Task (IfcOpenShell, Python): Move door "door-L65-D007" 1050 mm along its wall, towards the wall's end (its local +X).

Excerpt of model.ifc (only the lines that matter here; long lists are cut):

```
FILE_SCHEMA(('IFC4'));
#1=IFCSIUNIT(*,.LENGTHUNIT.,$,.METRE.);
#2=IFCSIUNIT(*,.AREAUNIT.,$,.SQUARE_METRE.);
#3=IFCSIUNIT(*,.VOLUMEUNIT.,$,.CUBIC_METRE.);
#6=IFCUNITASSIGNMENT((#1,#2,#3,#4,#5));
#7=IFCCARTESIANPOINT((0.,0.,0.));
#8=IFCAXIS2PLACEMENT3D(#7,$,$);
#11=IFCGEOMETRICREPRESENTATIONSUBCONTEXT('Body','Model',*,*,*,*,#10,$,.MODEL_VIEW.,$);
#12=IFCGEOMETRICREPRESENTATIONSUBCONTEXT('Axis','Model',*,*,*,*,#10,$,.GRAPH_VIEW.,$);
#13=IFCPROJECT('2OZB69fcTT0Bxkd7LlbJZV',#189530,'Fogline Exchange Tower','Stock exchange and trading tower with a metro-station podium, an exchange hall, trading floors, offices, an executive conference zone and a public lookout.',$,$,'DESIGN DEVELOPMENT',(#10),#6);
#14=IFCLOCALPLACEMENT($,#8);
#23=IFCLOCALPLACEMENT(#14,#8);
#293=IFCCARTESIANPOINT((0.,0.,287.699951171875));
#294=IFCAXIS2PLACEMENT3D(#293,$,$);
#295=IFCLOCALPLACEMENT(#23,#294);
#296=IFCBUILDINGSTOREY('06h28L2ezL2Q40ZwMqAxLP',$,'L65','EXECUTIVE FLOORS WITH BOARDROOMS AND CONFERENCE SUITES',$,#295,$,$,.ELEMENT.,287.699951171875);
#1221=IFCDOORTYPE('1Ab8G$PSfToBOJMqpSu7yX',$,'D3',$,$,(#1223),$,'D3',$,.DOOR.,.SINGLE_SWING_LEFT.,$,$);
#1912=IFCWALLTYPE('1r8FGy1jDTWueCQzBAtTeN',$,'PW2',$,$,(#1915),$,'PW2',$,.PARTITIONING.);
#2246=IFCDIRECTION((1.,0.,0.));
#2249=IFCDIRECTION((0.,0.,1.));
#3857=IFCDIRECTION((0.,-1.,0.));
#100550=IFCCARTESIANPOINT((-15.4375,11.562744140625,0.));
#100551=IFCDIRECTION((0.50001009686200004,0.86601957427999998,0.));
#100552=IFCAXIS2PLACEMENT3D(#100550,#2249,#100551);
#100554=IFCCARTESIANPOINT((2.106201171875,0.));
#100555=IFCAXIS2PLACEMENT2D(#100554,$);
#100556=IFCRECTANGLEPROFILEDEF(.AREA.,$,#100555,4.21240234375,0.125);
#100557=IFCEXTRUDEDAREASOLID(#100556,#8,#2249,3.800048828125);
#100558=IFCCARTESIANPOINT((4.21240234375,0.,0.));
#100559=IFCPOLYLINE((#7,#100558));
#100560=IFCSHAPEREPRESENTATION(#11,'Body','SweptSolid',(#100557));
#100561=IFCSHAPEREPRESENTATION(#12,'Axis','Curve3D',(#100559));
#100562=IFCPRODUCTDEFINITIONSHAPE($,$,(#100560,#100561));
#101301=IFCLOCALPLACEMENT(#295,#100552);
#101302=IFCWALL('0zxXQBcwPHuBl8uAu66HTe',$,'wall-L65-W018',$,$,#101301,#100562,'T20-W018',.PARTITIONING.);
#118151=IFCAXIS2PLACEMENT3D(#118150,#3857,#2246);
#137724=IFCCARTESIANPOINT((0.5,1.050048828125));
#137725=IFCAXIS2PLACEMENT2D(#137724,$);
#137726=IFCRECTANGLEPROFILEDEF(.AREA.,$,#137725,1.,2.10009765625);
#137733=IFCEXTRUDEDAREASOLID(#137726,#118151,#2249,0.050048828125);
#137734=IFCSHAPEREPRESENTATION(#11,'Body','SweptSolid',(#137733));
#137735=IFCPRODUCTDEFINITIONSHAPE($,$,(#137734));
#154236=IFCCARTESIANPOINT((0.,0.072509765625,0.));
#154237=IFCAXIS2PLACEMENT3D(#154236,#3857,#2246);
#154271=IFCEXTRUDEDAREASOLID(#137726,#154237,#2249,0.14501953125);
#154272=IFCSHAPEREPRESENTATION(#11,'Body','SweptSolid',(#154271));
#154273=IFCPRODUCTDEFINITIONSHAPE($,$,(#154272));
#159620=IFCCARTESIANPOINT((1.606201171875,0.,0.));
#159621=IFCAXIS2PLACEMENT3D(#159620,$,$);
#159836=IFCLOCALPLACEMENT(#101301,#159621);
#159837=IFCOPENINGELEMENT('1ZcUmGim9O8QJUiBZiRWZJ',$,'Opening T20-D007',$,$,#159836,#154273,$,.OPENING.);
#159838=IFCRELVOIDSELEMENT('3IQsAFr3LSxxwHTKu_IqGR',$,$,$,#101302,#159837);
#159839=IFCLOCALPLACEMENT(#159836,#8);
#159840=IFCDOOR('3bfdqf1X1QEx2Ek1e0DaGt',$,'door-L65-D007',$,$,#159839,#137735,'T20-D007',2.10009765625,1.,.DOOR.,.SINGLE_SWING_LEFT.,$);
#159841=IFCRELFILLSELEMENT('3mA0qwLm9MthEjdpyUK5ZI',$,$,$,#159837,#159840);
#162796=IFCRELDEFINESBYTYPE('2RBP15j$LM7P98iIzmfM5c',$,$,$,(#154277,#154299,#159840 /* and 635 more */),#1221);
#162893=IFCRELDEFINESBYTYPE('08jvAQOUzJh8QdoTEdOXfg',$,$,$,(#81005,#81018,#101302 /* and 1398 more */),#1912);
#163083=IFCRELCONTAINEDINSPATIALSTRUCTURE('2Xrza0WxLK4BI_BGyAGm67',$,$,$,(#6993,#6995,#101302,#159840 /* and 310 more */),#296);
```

```python
import ifcopenshell
import ifcopenshell.api.geometry
import ifcopenshell.util.placement
import ifcopenshell.util.unit

model = ifcopenshell.open("model.ifc")
unit_scale = ifcopenshell.util.unit.calculate_unit_scale(model)

door = model.by_id(159840)
opening = door.FillsVoids[0].RelatingOpeningElement
wall = opening.VoidsElements[0].RelatingBuildingElement

wall_matrix = ifcopenshell.util.placement.get_local_placement(wall.ObjectPlacement)
shift = wall_matrix[:3, 0] * 1.05 / unit_scale
before = ifcopenshell.util.placement.get_local_placement(door.ObjectPlacement)[:3, 3].copy()

# The door is placed relative to its opening, so it follows when the opening moves.
matrix = ifcopenshell.util.placement.get_local_placement(opening.ObjectPlacement)
matrix[:3, 3] += shift
ifcopenshell.api.geometry.edit_object_placement(
    model, product=opening, matrix=matrix, is_si=False, should_transform_children=True
)

after = ifcopenshell.util.placement.get_local_placement(door.ObjectPlacement)[:3, 3]
print("door moved by", (after - before).round(3) + 0.0)

model.write("model-out.ifc")
```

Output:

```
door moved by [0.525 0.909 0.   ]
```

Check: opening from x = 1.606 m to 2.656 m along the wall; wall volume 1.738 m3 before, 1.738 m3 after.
